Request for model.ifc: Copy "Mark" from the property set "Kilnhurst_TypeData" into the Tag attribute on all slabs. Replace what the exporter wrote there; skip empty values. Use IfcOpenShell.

First a look at what the model holds.

```python
import ifcopenshell
import ifcopenshell.util.element

model = ifcopenshell.open("model.ifc")
print(model.schema)
slabs = model.by_type("IfcSlab")
print(len(slabs), "slabs")
for e in slabs[:8]:
    source = ifcopenshell.util.element.get_pset(e, "Kilnhurst_TypeData", "Mark")
    target = e.Tag
    print(e.id(), repr(source), repr(target), sep=" | ")
```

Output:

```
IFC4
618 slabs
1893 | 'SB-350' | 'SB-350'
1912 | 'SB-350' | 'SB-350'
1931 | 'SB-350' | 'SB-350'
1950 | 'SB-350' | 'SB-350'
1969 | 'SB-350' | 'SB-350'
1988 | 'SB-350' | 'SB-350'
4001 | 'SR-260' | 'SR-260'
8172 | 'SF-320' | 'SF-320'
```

```python
import ifcopenshell
import ifcopenshell.util.element

model = ifcopenshell.open("model.ifc")

count = 0
for e in model.by_type("IfcSlab"):
    value = ifcopenshell.util.element.get_pset(e, "Kilnhurst_TypeData", "Mark")
    current = e.Tag
    if not value or not value.strip() or current == value:
        continue
    e.Tag = value
    count += 1

print(count, "slabs updated")

model.write("model-out.ifc")
```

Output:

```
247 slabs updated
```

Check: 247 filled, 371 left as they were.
